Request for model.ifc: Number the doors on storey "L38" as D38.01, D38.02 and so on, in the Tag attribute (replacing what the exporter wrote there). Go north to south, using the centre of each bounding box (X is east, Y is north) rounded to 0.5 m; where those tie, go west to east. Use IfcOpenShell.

First a look at what the model holds.

```python
import ifcopenshell
import ifcopenshell.util.element
import ifcopenshell.util.placement

model = ifcopenshell.open("model.ifc")
print(model.schema)
storey = next(s for s in model.by_type("IfcBuildingStorey") if s.Name == "L38")
doors = [e for e in ifcopenshell.util.element.get_decomposition(storey) if e.is_a("IfcDoor")]
for e in sorted(doors, key=lambda e: e.id()):
    origin = ifcopenshell.util.placement.get_local_placement(e.ObjectPlacement)[:3, 3]
    print(e.id(), e.Tag, e.Name, origin.round(2) + 0.0, sep=" | ")
```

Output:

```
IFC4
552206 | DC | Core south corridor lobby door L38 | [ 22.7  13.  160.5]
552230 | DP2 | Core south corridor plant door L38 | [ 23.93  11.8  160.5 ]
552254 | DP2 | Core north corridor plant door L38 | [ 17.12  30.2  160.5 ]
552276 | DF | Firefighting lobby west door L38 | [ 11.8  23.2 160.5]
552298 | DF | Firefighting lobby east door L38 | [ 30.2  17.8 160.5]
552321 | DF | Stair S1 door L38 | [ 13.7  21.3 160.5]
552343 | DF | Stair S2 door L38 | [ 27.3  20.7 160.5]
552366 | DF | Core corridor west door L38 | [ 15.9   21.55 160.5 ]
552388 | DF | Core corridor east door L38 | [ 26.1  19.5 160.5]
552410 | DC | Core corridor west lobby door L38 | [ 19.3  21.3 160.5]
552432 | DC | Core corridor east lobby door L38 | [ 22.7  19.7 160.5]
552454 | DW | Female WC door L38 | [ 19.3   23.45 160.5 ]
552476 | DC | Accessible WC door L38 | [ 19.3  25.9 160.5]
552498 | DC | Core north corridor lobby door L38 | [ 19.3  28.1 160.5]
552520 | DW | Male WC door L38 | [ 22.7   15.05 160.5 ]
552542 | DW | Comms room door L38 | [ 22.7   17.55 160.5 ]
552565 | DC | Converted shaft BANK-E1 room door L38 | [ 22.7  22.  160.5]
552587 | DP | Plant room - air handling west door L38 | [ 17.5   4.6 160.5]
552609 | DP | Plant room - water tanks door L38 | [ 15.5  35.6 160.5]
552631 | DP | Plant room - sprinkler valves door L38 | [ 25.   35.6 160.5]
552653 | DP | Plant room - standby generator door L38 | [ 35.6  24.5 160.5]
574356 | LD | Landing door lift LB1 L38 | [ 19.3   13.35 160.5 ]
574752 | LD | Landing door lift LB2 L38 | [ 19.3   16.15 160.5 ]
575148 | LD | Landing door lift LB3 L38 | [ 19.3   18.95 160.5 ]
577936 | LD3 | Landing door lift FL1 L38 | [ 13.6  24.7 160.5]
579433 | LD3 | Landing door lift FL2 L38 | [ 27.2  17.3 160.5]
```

```python
import ifcopenshell
import ifcopenshell.geom
import ifcopenshell.util.element
import ifcopenshell.util.shape

model = ifcopenshell.open("model.ifc")
settings = ifcopenshell.geom.settings()
settings.set("use-world-coords", True)


def centre(element):
    shape = ifcopenshell.geom.create_shape(settings, element)
    return ifcopenshell.util.shape.get_bbox_centroid(shape.geometry)


storey = next(s for s in model.by_type("IfcBuildingStorey") if s.Name == "L38")
doors = [e for e in ifcopenshell.util.element.get_decomposition(storey) if e.is_a("IfcDoor")]

# Insertion points can sit at a corner or the storey origin, so sort by the geometry (in metres).
centres = {e: centre(e) for e in doors}
doors.sort(key=lambda e: (-round(centres[e][1] / 0.5), centres[e][0]))

for i, e in enumerate(doors, start=1):
    number = f"D38.{i:02d}"
    e.Tag = number
    print(e.id(), number)

model.write("model-out.ifc")
```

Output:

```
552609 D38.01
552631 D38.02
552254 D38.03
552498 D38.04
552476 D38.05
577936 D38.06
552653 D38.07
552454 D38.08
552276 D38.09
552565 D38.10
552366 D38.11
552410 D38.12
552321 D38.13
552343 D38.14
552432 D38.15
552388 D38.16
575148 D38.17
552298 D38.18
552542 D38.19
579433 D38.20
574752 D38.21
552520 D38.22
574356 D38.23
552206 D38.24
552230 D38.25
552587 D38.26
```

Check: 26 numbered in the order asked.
